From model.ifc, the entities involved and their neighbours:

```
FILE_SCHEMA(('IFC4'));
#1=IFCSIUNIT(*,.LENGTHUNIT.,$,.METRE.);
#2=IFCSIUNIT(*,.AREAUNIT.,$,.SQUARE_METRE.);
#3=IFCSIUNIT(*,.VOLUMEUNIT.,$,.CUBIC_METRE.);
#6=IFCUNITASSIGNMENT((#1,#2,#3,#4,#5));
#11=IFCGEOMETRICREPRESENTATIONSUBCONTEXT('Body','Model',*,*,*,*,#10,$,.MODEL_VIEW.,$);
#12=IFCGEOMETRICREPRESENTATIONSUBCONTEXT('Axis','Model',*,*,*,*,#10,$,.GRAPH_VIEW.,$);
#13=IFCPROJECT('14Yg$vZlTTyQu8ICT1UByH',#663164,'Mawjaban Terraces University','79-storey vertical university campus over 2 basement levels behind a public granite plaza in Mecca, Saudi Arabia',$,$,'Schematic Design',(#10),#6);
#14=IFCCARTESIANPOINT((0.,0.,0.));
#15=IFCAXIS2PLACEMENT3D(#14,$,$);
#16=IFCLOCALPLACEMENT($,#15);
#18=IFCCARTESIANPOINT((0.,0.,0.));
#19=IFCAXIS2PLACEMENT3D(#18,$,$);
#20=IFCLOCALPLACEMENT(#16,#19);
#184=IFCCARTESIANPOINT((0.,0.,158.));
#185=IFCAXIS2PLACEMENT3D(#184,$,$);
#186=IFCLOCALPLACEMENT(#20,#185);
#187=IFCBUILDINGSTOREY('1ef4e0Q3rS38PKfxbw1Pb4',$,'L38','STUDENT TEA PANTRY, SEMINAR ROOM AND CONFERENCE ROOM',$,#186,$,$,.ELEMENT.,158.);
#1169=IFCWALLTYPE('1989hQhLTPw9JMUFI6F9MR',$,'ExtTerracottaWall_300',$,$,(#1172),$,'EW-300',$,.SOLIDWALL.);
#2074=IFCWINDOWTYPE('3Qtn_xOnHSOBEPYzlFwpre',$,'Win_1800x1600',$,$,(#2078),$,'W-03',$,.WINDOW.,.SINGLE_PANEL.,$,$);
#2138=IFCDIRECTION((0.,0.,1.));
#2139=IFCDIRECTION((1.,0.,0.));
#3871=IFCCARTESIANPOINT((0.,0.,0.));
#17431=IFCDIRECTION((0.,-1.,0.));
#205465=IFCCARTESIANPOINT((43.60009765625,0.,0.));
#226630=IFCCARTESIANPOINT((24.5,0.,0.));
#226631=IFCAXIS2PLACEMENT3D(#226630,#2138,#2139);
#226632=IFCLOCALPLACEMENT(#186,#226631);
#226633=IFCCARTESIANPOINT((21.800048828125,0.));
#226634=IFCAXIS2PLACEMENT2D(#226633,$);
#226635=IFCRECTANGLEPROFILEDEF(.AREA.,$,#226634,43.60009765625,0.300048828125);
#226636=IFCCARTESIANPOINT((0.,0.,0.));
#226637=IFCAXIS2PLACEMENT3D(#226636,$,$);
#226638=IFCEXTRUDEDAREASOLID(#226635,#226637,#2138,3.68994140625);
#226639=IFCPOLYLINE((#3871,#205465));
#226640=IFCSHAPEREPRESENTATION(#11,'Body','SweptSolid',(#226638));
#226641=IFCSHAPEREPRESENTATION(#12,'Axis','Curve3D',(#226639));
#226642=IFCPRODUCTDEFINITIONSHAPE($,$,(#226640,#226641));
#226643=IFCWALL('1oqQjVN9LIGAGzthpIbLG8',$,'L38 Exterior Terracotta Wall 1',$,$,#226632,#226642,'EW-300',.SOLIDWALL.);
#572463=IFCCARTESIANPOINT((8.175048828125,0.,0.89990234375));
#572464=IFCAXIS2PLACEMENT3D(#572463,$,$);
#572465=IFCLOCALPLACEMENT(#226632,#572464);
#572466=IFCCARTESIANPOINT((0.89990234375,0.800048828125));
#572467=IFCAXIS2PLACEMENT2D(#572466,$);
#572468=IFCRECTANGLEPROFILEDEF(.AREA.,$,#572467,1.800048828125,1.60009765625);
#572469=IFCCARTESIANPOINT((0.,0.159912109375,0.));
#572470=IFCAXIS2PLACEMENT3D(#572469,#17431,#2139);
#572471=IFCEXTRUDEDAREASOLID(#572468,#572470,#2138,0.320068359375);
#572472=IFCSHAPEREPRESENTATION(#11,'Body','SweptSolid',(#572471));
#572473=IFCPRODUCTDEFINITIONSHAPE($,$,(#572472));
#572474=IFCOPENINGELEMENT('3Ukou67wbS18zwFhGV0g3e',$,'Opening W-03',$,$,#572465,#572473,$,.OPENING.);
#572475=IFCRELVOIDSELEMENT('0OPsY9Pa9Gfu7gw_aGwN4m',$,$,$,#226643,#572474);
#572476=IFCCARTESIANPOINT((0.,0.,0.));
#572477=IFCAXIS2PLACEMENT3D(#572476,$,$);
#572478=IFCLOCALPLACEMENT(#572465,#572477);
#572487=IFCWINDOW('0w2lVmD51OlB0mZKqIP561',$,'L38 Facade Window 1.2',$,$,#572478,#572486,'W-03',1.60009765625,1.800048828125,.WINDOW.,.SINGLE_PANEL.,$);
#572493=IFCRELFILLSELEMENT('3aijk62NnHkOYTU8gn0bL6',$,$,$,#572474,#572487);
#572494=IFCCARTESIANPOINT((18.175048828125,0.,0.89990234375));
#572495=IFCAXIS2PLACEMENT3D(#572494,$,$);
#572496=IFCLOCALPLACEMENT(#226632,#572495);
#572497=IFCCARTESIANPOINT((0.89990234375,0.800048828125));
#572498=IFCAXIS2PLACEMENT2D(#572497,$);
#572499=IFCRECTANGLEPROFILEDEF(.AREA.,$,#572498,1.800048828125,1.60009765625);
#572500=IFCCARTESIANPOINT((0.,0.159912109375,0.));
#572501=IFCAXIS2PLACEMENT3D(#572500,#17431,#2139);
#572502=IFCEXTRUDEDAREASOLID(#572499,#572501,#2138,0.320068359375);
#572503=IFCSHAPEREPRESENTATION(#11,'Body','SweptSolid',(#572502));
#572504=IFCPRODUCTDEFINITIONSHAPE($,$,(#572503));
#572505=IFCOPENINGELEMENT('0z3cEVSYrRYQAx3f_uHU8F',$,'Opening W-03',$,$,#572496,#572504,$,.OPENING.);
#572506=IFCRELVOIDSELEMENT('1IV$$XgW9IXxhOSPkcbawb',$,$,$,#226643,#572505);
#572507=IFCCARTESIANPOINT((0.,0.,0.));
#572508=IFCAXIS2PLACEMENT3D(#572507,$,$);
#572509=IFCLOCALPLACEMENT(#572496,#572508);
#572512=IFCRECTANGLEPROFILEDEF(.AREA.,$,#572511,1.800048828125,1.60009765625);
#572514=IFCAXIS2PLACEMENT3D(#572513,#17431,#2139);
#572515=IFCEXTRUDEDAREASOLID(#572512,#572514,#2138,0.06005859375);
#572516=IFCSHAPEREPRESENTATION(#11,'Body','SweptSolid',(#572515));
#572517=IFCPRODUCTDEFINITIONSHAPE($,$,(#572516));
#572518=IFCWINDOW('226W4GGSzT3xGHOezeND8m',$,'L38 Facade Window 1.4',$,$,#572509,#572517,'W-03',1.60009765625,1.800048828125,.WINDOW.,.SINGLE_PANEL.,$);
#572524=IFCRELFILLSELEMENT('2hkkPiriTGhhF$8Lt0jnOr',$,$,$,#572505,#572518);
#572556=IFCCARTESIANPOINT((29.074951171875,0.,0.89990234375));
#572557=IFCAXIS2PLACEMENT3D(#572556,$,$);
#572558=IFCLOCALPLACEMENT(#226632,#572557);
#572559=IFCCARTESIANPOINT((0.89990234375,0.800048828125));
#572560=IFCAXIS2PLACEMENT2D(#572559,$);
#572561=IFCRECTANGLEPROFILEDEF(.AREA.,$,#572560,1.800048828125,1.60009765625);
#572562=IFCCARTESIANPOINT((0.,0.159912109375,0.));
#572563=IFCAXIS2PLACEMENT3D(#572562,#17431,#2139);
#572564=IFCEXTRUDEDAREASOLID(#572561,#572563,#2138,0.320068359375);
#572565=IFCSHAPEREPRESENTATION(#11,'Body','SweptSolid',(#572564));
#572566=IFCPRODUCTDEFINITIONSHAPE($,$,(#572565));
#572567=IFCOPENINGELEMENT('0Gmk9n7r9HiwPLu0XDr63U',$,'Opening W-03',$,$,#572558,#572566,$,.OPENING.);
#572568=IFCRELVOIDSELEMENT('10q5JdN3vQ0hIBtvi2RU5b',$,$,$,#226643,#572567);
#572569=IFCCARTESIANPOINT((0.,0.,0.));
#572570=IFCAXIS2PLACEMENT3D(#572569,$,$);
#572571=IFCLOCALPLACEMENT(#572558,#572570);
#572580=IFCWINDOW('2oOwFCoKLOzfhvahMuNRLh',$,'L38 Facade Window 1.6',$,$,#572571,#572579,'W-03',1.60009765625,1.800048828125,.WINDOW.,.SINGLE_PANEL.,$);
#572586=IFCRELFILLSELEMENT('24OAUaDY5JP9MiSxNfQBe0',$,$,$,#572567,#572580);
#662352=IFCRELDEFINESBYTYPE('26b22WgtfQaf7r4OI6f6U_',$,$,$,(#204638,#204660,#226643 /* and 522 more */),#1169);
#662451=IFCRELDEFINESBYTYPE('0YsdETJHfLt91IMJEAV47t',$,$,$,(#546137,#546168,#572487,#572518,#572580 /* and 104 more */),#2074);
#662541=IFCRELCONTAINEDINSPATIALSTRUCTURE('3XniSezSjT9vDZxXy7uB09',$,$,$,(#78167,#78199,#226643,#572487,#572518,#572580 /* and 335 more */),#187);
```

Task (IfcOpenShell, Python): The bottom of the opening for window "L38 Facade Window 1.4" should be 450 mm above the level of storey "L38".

```python
import numpy as np
import ifcopenshell
import ifcopenshell.api.geometry
import ifcopenshell.geom
import ifcopenshell.util.element
import ifcopenshell.util.placement
import ifcopenshell.util.shape
import ifcopenshell.util.unit

model = ifcopenshell.open("model.ifc")
unit_scale = ifcopenshell.util.unit.calculate_unit_scale(model)

window = model.by_guid("226W4GGSzT3xGHOezeND8m")
opening = window.FillsVoids[0].RelatingOpeningElement
storey = ifcopenshell.util.element.get_container(window, ifc_class="IfcBuildingStorey")
level = ifcopenshell.util.placement.get_local_placement(storey.ObjectPlacement)[2, 3]

# The opening's origin need not be at the sill, so measure its lowest point.
shape = ifcopenshell.geom.create_shape(ifcopenshell.geom.settings(), opening)
bottom = ifcopenshell.util.shape.get_shape_bottom_elevation(shape, shape.geometry) / unit_scale
dz = level + 0.45 - bottom

shift = np.array([0.0, 0.0, dz])
# The window is placed relative to its opening, so it follows when the opening moves.
matrix = ifcopenshell.util.placement.get_local_placement(opening.ObjectPlacement)
matrix[:3, 3] += shift
ifcopenshell.api.geometry.edit_object_placement(
    model, product=opening, matrix=matrix, is_si=False, should_transform_children=True
)

print(f"moved by {dz * unit_scale:+.3f} m")

model.write("model_v2.ifc")
```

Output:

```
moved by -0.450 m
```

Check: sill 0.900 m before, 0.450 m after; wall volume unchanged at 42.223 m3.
